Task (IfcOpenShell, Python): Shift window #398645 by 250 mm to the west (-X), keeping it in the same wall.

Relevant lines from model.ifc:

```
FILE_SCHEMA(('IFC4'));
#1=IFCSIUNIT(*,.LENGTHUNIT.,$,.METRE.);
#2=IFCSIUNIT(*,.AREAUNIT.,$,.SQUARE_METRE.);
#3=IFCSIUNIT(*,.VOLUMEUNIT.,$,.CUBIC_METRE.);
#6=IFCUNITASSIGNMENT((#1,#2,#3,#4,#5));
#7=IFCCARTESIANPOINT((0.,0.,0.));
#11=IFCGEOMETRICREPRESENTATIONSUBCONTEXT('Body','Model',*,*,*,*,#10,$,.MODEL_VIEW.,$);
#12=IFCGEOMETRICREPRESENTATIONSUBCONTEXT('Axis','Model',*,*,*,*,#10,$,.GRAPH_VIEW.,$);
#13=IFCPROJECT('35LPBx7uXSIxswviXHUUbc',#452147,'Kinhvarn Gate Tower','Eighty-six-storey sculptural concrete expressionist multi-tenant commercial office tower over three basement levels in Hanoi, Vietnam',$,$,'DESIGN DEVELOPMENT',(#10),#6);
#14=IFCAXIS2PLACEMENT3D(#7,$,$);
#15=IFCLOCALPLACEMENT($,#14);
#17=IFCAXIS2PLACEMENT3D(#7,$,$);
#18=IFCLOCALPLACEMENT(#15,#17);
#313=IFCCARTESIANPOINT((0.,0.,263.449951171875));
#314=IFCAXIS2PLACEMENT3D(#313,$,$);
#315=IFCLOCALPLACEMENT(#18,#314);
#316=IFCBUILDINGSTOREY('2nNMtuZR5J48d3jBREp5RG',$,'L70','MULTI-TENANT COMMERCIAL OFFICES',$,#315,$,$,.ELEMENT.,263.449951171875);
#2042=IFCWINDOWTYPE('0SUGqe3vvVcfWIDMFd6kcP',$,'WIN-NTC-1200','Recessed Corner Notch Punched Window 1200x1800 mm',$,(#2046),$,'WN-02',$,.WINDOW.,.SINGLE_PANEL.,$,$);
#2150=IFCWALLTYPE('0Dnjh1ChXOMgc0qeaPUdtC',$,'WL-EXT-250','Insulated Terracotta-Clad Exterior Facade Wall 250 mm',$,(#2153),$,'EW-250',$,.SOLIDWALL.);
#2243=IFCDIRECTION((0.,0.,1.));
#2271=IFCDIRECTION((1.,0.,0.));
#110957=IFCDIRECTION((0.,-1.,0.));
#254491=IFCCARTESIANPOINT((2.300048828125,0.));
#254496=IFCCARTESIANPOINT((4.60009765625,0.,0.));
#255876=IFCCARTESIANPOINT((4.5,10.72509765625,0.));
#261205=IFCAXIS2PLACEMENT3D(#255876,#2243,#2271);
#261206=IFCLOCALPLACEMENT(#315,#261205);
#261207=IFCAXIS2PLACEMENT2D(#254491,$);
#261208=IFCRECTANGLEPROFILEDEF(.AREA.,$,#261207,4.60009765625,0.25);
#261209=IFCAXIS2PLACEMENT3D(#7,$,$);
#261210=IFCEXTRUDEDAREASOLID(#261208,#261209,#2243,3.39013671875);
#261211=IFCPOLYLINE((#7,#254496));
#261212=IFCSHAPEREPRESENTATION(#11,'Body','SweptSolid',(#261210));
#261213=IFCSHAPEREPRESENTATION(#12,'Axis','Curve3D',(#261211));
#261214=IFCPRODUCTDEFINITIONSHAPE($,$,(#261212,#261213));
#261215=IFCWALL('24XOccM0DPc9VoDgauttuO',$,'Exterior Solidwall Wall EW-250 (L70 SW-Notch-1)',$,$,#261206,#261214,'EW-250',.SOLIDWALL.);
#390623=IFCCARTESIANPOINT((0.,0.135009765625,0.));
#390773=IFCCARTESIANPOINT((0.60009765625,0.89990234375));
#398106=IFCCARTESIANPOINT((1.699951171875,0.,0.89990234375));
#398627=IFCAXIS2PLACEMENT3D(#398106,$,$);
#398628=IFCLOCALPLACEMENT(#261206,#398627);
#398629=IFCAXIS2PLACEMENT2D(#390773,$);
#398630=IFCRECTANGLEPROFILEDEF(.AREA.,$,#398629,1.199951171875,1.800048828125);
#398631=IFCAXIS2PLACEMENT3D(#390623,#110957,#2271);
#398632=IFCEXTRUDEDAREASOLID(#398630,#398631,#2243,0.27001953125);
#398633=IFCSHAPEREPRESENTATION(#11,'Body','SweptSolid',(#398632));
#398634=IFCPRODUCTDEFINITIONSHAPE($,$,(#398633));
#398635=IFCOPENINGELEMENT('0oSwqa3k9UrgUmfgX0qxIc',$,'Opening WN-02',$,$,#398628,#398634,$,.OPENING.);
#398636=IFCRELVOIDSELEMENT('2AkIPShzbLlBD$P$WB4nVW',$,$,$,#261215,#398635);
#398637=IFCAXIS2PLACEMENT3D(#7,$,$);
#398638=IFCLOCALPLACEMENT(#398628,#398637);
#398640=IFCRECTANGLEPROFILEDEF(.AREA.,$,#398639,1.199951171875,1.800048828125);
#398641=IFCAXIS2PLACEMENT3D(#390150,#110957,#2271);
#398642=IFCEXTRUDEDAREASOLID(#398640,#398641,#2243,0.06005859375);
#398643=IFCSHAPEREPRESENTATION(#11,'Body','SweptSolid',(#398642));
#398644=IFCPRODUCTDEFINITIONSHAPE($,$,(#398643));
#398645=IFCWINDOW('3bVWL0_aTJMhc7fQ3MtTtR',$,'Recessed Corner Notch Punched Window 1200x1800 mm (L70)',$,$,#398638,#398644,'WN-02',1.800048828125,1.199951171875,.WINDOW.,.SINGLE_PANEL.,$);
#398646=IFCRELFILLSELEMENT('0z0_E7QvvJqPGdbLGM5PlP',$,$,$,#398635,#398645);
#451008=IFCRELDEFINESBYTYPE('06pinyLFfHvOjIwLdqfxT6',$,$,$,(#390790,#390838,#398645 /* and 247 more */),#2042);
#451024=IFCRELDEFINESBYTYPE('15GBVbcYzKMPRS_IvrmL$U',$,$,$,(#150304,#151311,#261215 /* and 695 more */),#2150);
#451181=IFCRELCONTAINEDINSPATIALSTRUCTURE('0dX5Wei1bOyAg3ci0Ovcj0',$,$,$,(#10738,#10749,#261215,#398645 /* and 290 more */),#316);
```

```python
import ifcopenshell
import ifcopenshell.api.geometry
import ifcopenshell.util.placement

model = ifcopenshell.open("model.ifc")

window = model.by_guid("3bVWL0_aTJMhc7fQ3MtTtR")
opening = window.FillsVoids[0].RelatingOpeningElement
wall = opening.VoidsElements[0].RelatingBuildingElement

wall_matrix = ifcopenshell.util.placement.get_local_placement(wall.ObjectPlacement)
shift = wall_matrix[:3, 0] * -0.25
before = ifcopenshell.util.placement.get_local_placement(window.ObjectPlacement)[:3, 3].copy()

# The window is placed relative to its opening, so it follows when the opening moves.
matrix = ifcopenshell.util.placement.get_local_placement(opening.ObjectPlacement)
matrix[:3, 3] += shift
ifcopenshell.api.geometry.edit_object_placement(
    model, product=opening, matrix=matrix, is_si=False, should_transform_children=True
)

after = ifcopenshell.util.placement.get_local_placement(window.ObjectPlacement)[:3, 3]
print("window moved by", (after - before).round(3) + 0.0)

model.write("model-out.ifc")
```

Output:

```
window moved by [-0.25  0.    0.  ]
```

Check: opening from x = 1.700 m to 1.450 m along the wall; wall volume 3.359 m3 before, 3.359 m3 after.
